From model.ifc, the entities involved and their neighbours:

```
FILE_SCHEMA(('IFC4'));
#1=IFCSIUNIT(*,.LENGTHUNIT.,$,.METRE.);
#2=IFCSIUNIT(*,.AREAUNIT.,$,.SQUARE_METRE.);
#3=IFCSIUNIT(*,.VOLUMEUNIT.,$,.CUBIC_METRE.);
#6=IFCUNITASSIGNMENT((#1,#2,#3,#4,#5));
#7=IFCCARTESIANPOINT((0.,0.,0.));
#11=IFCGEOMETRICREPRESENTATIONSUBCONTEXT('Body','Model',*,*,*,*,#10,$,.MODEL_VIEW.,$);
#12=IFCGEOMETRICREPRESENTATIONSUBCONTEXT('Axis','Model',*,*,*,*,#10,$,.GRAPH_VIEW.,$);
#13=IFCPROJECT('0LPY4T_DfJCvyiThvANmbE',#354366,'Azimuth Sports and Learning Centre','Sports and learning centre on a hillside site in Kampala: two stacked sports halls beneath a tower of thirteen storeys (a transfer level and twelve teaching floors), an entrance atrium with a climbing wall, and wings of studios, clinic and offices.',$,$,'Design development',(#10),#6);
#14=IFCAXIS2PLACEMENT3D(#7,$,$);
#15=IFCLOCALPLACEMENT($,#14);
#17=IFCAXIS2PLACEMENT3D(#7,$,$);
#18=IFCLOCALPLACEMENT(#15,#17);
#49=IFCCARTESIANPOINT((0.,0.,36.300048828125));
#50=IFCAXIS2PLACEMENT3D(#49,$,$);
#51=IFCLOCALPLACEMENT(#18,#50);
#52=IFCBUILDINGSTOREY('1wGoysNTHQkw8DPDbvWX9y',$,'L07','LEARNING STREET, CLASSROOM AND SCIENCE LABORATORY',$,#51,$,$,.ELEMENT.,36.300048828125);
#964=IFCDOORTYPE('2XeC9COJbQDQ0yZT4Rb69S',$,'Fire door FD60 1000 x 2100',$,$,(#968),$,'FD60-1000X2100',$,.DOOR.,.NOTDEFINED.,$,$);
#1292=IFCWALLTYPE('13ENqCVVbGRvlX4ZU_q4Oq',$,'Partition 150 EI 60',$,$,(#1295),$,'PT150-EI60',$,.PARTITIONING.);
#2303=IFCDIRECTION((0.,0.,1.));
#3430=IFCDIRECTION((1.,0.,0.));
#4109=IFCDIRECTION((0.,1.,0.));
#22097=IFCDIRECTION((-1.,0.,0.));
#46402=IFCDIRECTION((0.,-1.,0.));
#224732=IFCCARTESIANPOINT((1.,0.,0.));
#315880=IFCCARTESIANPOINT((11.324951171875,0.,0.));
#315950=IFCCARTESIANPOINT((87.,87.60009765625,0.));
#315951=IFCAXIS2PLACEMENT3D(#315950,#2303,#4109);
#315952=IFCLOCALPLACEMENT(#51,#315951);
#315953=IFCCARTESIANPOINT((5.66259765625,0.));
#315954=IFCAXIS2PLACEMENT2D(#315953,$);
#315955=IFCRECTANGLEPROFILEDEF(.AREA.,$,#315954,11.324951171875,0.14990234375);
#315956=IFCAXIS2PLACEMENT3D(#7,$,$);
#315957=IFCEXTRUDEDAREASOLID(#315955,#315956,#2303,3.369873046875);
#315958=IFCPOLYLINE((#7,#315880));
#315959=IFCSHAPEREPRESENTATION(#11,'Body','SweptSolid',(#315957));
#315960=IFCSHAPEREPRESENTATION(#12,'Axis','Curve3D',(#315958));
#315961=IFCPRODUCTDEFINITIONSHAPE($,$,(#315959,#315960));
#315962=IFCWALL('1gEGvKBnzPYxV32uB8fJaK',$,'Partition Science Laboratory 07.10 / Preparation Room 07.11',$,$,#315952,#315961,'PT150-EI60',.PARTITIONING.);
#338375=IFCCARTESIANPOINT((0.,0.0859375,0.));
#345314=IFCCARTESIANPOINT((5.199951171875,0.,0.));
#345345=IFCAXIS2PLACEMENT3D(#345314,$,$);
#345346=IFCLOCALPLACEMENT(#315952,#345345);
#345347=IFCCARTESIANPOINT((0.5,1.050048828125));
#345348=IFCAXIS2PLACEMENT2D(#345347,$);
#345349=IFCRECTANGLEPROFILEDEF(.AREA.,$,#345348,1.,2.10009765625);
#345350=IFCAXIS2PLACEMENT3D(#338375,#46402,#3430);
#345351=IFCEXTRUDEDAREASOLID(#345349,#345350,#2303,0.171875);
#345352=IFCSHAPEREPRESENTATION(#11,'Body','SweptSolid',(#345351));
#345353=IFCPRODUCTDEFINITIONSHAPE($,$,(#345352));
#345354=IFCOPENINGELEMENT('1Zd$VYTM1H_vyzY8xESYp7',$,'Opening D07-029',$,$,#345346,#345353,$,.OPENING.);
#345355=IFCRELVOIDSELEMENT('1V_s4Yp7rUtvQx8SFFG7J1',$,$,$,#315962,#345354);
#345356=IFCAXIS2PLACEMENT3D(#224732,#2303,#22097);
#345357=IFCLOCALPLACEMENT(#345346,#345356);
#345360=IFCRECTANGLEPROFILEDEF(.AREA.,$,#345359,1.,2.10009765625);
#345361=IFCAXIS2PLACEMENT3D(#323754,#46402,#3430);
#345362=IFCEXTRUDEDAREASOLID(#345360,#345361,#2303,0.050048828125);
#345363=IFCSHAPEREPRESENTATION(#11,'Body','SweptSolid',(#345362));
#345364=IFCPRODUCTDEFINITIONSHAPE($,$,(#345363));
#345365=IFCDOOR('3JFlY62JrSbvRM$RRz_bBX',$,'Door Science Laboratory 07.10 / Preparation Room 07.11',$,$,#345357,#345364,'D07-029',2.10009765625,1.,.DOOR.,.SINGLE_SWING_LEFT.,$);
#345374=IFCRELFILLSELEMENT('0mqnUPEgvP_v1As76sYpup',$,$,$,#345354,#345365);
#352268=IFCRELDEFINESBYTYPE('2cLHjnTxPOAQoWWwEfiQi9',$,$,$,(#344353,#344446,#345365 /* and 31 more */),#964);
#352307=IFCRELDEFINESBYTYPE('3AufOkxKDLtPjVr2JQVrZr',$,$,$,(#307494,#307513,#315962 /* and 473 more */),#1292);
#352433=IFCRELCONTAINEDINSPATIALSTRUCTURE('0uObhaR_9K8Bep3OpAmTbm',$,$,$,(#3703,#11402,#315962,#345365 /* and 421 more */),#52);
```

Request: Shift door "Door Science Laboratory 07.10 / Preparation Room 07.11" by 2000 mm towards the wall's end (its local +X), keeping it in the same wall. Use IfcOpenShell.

```python
import ifcopenshell
import ifcopenshell.api.geometry
import ifcopenshell.util.placement

model = ifcopenshell.open("model.ifc")

door = model.by_id(345365)
opening = door.FillsVoids[0].RelatingOpeningElement
wall = opening.VoidsElements[0].RelatingBuildingElement

wall_matrix = ifcopenshell.util.placement.get_local_placement(wall.ObjectPlacement)
shift = wall_matrix[:3, 0] * 2.0
before = ifcopenshell.util.placement.get_local_placement(door.ObjectPlacement)[:3, 3].copy()

# The door is placed relative to its opening, so it follows when the opening moves.
matrix = ifcopenshell.util.placement.get_local_placement(opening.ObjectPlacement)
matrix[:3, 3] += shift
ifcopenshell.api.geometry.edit_object_placement(
    model, product=opening, matrix=matrix, is_si=False, should_transform_children=True
)

after = ifcopenshell.util.placement.get_local_placement(door.ObjectPlacement)[:3, 3]
print("door moved by", (after - before).round(3) + 0.0)

model.write("model-out.ifc")
```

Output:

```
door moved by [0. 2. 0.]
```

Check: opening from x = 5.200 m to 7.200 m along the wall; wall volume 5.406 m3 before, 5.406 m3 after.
